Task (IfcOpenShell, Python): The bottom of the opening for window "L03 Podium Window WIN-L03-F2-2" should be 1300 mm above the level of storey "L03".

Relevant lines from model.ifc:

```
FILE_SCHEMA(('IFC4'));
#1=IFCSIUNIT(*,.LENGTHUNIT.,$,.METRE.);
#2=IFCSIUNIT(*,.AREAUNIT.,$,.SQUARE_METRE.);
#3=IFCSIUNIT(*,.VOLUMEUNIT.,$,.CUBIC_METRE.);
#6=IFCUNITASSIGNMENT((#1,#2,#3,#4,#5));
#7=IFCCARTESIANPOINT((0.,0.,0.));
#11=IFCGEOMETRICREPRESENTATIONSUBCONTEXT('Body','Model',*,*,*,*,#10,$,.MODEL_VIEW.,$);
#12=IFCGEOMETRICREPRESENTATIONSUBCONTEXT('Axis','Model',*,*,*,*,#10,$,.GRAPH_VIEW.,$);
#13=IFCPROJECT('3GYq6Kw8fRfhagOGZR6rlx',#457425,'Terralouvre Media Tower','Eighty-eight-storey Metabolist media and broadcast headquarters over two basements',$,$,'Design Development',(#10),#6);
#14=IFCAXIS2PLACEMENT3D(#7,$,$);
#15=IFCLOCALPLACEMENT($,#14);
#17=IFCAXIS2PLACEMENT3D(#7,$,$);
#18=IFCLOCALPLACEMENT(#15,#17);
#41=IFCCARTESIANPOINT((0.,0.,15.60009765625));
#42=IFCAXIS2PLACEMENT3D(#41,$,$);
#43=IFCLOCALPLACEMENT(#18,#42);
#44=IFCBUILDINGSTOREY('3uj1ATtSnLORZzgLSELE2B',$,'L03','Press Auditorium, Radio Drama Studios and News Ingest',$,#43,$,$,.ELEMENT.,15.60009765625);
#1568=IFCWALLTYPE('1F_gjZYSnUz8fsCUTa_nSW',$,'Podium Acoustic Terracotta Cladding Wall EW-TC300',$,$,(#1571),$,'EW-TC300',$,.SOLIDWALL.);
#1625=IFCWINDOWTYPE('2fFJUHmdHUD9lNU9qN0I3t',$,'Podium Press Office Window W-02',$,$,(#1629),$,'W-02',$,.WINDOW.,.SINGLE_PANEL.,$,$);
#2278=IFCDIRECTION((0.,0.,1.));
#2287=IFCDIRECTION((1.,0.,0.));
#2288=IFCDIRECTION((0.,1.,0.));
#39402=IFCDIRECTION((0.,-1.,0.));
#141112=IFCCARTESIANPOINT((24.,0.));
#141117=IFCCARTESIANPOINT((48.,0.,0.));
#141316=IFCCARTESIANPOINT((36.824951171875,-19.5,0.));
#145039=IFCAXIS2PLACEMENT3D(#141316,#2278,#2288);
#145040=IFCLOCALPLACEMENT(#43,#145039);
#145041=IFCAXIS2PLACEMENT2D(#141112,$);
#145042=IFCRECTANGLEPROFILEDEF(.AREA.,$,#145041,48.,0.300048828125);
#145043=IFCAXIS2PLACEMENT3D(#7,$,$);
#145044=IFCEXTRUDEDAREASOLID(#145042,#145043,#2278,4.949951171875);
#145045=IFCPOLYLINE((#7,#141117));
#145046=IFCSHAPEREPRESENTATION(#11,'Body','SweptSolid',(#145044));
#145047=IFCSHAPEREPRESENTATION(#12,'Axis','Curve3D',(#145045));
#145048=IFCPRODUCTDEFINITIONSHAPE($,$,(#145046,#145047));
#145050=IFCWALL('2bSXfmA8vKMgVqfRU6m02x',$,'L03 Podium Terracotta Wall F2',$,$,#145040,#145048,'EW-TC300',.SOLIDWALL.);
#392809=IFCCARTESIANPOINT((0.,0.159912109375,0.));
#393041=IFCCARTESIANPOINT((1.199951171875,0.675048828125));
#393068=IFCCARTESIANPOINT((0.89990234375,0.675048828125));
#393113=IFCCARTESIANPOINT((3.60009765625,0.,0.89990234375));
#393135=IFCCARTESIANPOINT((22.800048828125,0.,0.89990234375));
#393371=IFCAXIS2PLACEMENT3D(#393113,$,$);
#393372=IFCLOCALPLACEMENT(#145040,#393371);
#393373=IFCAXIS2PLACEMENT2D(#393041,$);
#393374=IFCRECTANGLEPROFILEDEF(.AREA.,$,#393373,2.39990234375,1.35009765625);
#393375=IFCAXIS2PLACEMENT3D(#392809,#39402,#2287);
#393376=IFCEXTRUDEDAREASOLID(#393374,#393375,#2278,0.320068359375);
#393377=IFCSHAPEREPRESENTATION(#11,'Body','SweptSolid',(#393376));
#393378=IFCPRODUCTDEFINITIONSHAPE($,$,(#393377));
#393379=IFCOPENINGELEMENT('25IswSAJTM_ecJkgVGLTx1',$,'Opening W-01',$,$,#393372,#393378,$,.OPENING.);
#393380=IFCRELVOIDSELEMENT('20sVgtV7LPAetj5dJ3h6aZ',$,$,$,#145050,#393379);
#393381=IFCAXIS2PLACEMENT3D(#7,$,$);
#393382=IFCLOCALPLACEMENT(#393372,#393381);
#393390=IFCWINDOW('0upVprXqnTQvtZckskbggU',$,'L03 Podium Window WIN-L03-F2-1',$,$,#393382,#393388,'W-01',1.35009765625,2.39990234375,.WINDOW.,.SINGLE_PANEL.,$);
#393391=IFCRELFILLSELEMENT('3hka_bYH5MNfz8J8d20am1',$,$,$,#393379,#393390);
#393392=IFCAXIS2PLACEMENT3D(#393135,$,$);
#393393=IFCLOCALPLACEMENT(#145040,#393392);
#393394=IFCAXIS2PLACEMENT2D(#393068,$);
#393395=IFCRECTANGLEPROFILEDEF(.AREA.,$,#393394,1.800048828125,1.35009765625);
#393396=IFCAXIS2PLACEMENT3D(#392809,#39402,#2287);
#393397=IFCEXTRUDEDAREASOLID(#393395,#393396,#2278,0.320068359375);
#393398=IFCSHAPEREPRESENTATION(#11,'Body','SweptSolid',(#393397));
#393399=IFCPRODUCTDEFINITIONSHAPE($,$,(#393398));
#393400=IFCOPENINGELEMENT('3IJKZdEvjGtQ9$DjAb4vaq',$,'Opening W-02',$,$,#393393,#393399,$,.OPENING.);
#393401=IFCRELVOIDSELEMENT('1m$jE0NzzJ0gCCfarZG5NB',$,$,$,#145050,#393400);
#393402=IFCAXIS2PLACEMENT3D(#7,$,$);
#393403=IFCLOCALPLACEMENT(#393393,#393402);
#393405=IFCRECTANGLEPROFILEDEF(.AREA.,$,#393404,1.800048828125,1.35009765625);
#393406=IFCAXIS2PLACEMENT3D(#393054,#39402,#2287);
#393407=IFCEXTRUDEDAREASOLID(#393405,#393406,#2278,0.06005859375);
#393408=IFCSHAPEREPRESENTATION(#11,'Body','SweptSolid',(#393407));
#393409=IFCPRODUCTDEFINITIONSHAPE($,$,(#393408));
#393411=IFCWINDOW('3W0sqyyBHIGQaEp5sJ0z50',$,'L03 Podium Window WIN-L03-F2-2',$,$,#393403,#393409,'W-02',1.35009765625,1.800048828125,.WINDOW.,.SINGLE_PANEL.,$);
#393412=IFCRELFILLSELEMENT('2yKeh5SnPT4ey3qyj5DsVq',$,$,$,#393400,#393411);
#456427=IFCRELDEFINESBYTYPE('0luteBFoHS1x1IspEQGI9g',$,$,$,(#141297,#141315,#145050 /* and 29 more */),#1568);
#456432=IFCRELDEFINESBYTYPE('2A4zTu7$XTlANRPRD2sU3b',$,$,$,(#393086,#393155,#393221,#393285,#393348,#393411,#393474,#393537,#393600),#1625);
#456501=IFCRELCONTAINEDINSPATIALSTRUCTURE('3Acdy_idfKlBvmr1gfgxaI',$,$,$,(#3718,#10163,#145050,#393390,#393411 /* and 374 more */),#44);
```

```python
import numpy as np
import ifcopenshell
import ifcopenshell.api.geometry
import ifcopenshell.geom
import ifcopenshell.util.element
import ifcopenshell.util.placement
import ifcopenshell.util.shape
import ifcopenshell.util.unit

model = ifcopenshell.open("model.ifc")
unit_scale = ifcopenshell.util.unit.calculate_unit_scale(model)

window = model.by_id(393411)
opening = window.FillsVoids[0].RelatingOpeningElement
storey = ifcopenshell.util.element.get_container(window, ifc_class="IfcBuildingStorey")
level = ifcopenshell.util.placement.get_local_placement(storey.ObjectPlacement)[2, 3]

# The opening's origin need not be at the sill, so measure its lowest point.
shape = ifcopenshell.geom.create_shape(ifcopenshell.geom.settings(), opening)
bottom = ifcopenshell.util.shape.get_shape_bottom_elevation(shape, shape.geometry) / unit_scale
dz = level + 1.3 - bottom

shift = np.array([0.0, 0.0, dz])
# The window is placed relative to its opening, so it follows when the opening moves.
matrix = ifcopenshell.util.placement.get_local_placement(opening.ObjectPlacement)
matrix[:3, 3] += shift
ifcopenshell.api.geometry.edit_object_placement(
    model, product=opening, matrix=matrix, is_si=False, should_transform_children=True
)

print(f"moved by {dz * unit_scale:+.3f} m")

model.write("model_rev.ifc")
```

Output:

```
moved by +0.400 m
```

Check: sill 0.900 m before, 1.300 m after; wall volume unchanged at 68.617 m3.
